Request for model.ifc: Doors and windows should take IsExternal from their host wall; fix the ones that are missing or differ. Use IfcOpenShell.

First a look at what the model holds.

```python
import ifcopenshell
import ifcopenshell.util.element

model = ifcopenshell.open("model.ifc")
print(model.schema)
seen = {}
for e in model.by_type("IfcDoor") + model.by_type("IfcWindow"):
    if not e.FillsVoids:
        continue
    host = e.FillsVoids[0].RelatingOpeningElement.VoidsElements[0].RelatingBuildingElement
    own = ifcopenshell.util.element.get_pset(e, f"Pset_{e.is_a()[3:].removesuffix('StandardCase')}Common", "IsExternal")
    wall = ifcopenshell.util.element.get_pset(host, "Pset_WallCommon", "IsExternal")
    seen[e.is_a(), own, wall] = seen.get((e.is_a(), own, wall), 0) + 1
for (cls, own, wall), count in sorted(seen.items(), key=str):
    print(count, cls, "IsExternal:", own, "| host wall:", wall)
```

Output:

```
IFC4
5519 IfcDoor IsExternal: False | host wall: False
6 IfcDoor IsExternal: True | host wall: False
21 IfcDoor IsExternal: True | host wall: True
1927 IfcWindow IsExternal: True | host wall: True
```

```python
import ifcopenshell
import ifcopenshell.api.pset
import ifcopenshell.util.element

model = ifcopenshell.open("model.ifc")

count = 0
for ifc_class, pset_name in (("IfcDoor", "Pset_DoorCommon"), ("IfcWindow", "Pset_WindowCommon")):
    for e in model.by_type(ifc_class):
        if not e.FillsVoids:
            continue
        host = e.FillsVoids[0].RelatingOpeningElement.VoidsElements[0].RelatingBuildingElement
        external = ifcopenshell.util.element.get_pset(host, "Pset_WallCommon", "IsExternal")
        if external is None or ifcopenshell.util.element.get_pset(e, pset_name, "IsExternal") == external:
            continue
        pset = ifcopenshell.api.pset.add_pset(model, product=e, name=pset_name)
        ifcopenshell.api.pset.edit_pset(model, pset=pset, properties={"IsExternal": external})
        count += 1

print(count, "updated")

model.write("model_updated.ifc")
```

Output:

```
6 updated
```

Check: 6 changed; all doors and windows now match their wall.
